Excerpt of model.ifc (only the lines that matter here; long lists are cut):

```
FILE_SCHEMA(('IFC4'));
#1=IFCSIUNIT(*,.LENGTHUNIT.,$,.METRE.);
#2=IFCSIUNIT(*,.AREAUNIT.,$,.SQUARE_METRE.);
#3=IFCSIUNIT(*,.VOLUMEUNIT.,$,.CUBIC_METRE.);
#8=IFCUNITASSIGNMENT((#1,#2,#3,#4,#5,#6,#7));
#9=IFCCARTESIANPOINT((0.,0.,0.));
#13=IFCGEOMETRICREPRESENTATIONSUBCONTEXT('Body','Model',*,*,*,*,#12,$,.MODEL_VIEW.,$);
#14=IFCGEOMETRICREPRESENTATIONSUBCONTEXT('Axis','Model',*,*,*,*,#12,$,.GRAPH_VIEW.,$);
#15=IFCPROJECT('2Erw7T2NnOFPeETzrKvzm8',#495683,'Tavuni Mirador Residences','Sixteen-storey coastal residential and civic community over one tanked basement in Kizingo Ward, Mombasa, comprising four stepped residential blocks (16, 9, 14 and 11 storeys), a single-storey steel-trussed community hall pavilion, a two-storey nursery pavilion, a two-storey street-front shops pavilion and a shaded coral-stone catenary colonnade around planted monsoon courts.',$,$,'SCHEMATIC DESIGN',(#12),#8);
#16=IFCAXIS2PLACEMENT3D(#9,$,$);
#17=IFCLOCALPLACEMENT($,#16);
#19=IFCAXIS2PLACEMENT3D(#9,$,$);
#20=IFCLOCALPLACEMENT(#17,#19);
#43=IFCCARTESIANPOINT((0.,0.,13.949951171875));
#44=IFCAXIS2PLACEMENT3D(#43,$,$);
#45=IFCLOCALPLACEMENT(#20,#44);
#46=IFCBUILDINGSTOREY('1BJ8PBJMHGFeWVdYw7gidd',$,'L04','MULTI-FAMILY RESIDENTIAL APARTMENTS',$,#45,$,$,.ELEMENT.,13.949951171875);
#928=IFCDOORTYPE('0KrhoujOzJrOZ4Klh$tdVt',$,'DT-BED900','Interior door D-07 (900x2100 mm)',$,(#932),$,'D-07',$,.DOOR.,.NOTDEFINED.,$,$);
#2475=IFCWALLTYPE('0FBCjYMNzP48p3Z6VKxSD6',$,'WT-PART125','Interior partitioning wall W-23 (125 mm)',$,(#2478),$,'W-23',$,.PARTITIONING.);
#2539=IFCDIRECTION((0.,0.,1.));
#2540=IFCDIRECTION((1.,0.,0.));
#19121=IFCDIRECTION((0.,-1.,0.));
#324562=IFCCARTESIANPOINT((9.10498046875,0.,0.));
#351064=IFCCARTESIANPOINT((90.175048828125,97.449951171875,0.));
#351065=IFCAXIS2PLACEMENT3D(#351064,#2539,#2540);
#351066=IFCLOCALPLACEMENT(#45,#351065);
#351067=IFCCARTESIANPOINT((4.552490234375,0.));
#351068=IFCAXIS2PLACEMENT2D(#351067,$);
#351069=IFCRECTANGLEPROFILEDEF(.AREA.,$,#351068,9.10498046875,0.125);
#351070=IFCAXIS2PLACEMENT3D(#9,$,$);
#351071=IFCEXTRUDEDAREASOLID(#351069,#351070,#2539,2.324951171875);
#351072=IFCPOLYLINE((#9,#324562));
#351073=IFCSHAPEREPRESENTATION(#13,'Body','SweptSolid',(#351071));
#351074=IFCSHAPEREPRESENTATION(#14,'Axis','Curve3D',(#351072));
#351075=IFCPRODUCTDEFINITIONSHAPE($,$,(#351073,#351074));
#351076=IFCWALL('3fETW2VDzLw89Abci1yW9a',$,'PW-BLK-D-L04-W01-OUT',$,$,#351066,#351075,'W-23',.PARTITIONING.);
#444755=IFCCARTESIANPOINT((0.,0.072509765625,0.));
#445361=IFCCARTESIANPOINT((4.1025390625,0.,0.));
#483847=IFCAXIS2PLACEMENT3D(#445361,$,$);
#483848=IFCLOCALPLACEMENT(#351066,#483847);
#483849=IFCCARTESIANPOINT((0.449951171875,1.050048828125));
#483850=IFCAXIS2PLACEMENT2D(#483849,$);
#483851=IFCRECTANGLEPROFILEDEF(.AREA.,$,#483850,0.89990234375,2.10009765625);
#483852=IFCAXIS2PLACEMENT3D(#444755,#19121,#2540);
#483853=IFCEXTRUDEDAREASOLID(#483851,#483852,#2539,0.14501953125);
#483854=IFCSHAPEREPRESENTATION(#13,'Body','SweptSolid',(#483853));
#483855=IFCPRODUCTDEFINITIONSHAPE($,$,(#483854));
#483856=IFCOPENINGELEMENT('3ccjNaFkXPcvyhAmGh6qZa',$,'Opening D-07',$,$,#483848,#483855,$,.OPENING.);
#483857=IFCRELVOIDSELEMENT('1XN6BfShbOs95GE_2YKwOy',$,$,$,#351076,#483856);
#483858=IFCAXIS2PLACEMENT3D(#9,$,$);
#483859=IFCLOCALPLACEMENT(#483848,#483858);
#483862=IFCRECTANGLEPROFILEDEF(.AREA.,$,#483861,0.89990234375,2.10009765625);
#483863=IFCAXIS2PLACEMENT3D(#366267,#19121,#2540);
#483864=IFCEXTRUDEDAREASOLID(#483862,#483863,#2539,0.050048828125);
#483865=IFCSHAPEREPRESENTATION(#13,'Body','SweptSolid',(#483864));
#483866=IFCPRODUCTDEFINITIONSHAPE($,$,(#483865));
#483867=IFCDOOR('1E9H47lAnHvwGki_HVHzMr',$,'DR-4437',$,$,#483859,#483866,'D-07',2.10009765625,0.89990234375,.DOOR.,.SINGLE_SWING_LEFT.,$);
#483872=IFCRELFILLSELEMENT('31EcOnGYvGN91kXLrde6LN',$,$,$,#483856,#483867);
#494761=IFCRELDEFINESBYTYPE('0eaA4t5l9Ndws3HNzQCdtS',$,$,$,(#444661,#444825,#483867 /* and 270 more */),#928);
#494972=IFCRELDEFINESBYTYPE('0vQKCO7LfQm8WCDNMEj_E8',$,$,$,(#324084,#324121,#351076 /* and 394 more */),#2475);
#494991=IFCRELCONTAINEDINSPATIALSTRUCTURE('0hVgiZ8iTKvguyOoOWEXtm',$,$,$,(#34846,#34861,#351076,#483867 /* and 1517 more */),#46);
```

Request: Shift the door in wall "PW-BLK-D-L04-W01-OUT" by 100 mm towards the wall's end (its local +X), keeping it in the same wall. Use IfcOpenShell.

```python
import ifcopenshell
import ifcopenshell.api.geometry
import ifcopenshell.util.placement

model = ifcopenshell.open("model.ifc")

door = model.by_guid("1E9H47lAnHvwGki_HVHzMr")
opening = door.FillsVoids[0].RelatingOpeningElement
wall = opening.VoidsElements[0].RelatingBuildingElement

wall_matrix = ifcopenshell.util.placement.get_local_placement(wall.ObjectPlacement)
shift = wall_matrix[:3, 0] * 0.1
before = ifcopenshell.util.placement.get_local_placement(door.ObjectPlacement)[:3, 3].copy()

# The door is placed relative to its opening, so it follows when the opening moves.
matrix = ifcopenshell.util.placement.get_local_placement(opening.ObjectPlacement)
matrix[:3, 3] += shift
ifcopenshell.api.geometry.edit_object_placement(
    model, product=opening, matrix=matrix, is_si=False, should_transform_children=True
)

after = ifcopenshell.util.placement.get_local_placement(door.ObjectPlacement)[:3, 3]
print("door moved by", (after - before).round(3) + 0.0)

model.write("model_v2.ifc")
```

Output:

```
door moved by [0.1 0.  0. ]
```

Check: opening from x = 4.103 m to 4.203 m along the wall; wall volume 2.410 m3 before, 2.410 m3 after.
